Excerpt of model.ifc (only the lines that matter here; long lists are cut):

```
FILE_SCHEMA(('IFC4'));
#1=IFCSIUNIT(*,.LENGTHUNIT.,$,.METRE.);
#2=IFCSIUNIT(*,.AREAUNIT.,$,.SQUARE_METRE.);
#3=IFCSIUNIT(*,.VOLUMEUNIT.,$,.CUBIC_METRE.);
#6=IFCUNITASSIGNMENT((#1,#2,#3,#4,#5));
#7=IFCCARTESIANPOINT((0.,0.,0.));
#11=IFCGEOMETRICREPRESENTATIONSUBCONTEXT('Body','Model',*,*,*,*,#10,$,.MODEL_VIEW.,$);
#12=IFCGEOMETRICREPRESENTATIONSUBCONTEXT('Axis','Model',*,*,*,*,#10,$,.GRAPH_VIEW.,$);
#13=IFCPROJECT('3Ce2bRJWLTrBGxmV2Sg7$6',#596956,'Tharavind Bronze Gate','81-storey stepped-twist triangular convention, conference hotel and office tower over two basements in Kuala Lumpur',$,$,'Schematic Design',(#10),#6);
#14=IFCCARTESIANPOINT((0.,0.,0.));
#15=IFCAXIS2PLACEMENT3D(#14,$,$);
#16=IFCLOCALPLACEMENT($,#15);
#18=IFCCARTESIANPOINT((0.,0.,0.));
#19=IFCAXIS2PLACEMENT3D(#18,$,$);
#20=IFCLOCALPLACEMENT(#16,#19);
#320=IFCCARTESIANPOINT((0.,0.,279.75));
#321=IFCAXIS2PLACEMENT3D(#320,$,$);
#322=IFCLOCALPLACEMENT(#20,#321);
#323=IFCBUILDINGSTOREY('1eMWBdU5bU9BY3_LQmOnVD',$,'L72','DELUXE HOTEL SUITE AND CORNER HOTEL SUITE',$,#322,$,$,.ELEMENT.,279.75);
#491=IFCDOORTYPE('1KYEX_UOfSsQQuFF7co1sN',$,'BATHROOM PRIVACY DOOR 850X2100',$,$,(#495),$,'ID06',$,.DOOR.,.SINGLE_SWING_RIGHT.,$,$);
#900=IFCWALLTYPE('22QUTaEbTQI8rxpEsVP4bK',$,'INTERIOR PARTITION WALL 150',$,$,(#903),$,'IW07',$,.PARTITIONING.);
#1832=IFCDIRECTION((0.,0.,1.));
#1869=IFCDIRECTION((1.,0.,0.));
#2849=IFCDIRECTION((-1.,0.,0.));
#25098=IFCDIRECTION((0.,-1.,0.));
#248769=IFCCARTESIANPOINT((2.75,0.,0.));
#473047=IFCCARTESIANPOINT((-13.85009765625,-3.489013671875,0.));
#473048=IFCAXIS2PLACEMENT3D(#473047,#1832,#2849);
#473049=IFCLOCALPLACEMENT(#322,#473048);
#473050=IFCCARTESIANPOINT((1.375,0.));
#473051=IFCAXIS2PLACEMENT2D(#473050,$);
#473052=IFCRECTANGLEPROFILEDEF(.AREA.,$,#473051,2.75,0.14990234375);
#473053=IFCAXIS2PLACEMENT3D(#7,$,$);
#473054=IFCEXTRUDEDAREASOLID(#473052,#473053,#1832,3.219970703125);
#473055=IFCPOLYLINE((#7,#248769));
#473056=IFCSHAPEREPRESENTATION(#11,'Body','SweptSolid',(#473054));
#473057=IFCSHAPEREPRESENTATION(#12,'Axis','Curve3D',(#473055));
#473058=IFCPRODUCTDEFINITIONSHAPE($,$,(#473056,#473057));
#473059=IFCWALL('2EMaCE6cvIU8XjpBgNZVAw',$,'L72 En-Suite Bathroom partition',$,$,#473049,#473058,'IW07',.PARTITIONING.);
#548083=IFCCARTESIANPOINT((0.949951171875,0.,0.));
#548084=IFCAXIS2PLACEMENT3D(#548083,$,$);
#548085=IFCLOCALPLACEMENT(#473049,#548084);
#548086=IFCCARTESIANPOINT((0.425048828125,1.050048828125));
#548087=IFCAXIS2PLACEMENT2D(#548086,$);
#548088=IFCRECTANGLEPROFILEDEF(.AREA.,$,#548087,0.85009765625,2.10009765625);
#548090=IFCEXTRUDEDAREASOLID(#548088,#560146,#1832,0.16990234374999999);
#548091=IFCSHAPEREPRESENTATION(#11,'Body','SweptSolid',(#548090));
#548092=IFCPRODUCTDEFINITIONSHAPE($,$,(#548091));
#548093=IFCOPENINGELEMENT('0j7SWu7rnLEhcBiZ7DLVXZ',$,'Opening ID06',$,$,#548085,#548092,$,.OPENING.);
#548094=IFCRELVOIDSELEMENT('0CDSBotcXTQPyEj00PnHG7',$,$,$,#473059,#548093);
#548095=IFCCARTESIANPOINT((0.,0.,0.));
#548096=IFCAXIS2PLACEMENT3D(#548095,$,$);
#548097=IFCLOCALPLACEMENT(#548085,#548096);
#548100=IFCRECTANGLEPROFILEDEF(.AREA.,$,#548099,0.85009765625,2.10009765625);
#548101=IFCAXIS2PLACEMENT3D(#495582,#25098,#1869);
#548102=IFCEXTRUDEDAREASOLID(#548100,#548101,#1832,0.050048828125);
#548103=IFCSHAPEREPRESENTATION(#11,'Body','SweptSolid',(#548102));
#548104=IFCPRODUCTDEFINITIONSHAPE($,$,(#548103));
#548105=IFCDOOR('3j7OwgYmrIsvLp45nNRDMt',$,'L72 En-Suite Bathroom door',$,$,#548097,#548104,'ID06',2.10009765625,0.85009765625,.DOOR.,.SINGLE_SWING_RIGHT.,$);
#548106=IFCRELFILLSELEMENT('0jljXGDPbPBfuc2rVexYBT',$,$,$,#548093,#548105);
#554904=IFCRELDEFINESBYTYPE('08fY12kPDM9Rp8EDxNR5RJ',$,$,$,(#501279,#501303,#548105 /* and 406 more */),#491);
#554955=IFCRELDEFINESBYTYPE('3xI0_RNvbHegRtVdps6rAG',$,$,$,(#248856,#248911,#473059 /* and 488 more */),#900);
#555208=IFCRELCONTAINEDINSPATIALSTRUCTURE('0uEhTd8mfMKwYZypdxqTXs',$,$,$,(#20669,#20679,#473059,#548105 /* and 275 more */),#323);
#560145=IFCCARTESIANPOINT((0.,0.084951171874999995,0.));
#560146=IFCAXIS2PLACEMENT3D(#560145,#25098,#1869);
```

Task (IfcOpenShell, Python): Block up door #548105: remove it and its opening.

```python
import ifcopenshell
import ifcopenshell.api.feature
import ifcopenshell.api.root
import ifcopenshell.geom
import ifcopenshell.util.shape

model = ifcopenshell.open("model.ifc")
settings = ifcopenshell.geom.settings()


def volume(element):
    """Net volume in cubic metres, openings subtracted."""
    shape = ifcopenshell.geom.create_shape(settings, element)
    return ifcopenshell.util.shape.get_volume(shape.geometry)


door = model.by_guid("3j7OwgYmrIsvLp45nNRDMt")
opening = door.FillsVoids[0].RelatingOpeningElement
wall = opening.VoidsElements[0].RelatingBuildingElement
before = volume(wall)

ifcopenshell.api.root.remove_product(model, product=door)
ifcopenshell.api.feature.remove_feature(model, feature=opening)

after = volume(wall)

print(f"wall volume {before:.3f} -> {after:.3f} m3")

model.write("model_rev.ifc")
```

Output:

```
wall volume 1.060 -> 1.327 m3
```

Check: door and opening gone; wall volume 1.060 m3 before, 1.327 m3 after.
